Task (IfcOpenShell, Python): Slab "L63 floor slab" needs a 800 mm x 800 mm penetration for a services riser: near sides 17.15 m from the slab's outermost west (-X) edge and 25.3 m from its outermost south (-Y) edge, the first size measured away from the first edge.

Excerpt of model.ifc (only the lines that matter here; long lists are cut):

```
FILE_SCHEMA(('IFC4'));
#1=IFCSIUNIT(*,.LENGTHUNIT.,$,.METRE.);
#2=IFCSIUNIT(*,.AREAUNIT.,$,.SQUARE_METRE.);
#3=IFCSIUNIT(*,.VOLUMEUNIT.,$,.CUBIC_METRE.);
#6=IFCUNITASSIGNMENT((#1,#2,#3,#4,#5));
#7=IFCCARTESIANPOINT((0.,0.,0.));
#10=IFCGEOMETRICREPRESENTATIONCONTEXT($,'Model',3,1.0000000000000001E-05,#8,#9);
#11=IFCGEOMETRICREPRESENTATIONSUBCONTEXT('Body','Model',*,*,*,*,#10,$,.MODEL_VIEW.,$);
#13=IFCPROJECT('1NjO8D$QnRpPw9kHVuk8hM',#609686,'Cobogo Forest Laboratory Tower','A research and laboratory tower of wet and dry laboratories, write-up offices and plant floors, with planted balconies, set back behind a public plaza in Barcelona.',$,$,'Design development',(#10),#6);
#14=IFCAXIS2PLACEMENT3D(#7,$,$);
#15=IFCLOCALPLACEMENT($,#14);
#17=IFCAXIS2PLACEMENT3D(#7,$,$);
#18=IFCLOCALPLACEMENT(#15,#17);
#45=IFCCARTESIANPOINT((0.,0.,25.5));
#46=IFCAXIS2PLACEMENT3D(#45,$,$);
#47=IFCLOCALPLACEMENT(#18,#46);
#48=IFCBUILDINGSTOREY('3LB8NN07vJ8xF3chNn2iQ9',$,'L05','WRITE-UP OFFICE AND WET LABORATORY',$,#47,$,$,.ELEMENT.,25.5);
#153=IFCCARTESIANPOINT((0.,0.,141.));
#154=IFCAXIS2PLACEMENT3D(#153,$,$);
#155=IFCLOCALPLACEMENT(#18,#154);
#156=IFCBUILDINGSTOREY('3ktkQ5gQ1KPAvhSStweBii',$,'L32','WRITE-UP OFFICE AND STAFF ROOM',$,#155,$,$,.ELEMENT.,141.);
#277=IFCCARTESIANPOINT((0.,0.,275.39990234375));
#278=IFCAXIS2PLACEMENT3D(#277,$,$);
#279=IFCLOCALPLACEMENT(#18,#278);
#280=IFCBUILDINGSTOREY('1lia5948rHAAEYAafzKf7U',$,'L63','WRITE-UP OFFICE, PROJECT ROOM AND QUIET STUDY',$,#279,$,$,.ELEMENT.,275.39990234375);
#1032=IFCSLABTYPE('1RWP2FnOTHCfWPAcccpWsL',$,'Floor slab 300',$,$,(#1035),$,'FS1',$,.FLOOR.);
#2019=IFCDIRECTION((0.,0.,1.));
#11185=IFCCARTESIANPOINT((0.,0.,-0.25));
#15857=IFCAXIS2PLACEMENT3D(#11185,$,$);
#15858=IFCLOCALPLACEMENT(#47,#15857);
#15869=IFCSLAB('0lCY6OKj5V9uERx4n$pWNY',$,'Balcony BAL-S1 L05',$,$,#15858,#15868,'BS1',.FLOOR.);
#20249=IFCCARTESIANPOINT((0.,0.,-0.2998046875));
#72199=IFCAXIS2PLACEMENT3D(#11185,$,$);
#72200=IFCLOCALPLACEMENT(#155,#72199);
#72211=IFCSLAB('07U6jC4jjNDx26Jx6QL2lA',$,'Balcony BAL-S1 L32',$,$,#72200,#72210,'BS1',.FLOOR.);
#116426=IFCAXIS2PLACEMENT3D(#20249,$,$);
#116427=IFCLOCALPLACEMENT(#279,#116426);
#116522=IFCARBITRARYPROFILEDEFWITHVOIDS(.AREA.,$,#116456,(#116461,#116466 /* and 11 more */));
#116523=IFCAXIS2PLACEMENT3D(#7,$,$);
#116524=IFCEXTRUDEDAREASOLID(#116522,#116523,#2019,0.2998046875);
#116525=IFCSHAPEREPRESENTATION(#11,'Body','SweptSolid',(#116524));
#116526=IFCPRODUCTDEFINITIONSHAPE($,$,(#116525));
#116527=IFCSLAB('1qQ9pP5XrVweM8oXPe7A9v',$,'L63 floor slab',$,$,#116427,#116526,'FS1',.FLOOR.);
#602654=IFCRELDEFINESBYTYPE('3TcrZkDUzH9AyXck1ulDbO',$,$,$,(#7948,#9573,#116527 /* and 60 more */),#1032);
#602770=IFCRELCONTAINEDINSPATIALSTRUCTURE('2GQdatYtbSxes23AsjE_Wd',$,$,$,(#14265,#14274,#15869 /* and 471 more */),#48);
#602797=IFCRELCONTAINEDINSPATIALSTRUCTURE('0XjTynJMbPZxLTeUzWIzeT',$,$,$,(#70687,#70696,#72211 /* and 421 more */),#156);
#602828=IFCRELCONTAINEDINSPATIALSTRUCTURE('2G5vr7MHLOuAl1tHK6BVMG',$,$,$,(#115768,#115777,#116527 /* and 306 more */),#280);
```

```python
import numpy as np
import ifcopenshell
import ifcopenshell.api.feature
import ifcopenshell.api.geometry
import ifcopenshell.api.root
import ifcopenshell.geom
import ifcopenshell.util.placement
import ifcopenshell.util.representation
import ifcopenshell.util.shape
import ifcopenshell.util.unit

model = ifcopenshell.open("model.ifc")
unit_scale = ifcopenshell.util.unit.calculate_unit_scale(model)
settings = ifcopenshell.geom.settings()


def volume(element):
    """Net volume in cubic metres, openings subtracted."""
    shape = ifcopenshell.geom.create_shape(settings, element)
    return ifcopenshell.util.shape.get_volume(shape.geometry)


slab = model.by_guid("1qQ9pP5XrVweM8oXPe7A9v")
before = volume(slab)

# Extent in the slab's own axes, in metres. The edges named are its -X and -Y sides.
slab_shape = ifcopenshell.geom.create_shape(settings, slab)
vertices = ifcopenshell.util.shape.get_vertices(slab_shape.geometry)
x_min, y_min, bottom = vertices.min(axis=0)
top = vertices[:, 2].max()

opening = ifcopenshell.api.root.create_entity(model, ifc_class="IfcOpeningElement", name="Services riser opening", predefined_type="OPENING")
context = ifcopenshell.util.representation.get_context(model, "Model", "Body", "MODEL_VIEW")
width, depth = 0.8, 0.8
outline = [(0.0, 0.0), (width, 0.0), (width, depth), (0.0, depth), (0.0, 0.0)]
# Overshoot both faces by 50 mm so the cut is clean.
shape = ifcopenshell.api.geometry.add_slab_representation(
    model, context=context, depth=top - bottom + 0.1, polyline=outline
)
ifcopenshell.api.geometry.assign_representation(model, product=opening, representation=shape)

matrix = ifcopenshell.util.placement.get_local_placement(slab.ObjectPlacement)
matrix[:, 3] = matrix @ np.append(np.array([x_min + 17.15, y_min + 25.3, bottom - 0.05]) / unit_scale, 1.0)
ifcopenshell.api.geometry.edit_object_placement(model, product=opening, matrix=matrix, is_si=False)
ifcopenshell.api.feature.add_feature(model, feature=opening, element=slab)

after = volume(slab)

print(f"slab volume {before:.3f} -> {after:.3f} m3")

model.write("model_edited.ifc")
```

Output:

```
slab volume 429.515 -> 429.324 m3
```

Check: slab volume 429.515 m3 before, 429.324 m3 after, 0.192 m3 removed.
